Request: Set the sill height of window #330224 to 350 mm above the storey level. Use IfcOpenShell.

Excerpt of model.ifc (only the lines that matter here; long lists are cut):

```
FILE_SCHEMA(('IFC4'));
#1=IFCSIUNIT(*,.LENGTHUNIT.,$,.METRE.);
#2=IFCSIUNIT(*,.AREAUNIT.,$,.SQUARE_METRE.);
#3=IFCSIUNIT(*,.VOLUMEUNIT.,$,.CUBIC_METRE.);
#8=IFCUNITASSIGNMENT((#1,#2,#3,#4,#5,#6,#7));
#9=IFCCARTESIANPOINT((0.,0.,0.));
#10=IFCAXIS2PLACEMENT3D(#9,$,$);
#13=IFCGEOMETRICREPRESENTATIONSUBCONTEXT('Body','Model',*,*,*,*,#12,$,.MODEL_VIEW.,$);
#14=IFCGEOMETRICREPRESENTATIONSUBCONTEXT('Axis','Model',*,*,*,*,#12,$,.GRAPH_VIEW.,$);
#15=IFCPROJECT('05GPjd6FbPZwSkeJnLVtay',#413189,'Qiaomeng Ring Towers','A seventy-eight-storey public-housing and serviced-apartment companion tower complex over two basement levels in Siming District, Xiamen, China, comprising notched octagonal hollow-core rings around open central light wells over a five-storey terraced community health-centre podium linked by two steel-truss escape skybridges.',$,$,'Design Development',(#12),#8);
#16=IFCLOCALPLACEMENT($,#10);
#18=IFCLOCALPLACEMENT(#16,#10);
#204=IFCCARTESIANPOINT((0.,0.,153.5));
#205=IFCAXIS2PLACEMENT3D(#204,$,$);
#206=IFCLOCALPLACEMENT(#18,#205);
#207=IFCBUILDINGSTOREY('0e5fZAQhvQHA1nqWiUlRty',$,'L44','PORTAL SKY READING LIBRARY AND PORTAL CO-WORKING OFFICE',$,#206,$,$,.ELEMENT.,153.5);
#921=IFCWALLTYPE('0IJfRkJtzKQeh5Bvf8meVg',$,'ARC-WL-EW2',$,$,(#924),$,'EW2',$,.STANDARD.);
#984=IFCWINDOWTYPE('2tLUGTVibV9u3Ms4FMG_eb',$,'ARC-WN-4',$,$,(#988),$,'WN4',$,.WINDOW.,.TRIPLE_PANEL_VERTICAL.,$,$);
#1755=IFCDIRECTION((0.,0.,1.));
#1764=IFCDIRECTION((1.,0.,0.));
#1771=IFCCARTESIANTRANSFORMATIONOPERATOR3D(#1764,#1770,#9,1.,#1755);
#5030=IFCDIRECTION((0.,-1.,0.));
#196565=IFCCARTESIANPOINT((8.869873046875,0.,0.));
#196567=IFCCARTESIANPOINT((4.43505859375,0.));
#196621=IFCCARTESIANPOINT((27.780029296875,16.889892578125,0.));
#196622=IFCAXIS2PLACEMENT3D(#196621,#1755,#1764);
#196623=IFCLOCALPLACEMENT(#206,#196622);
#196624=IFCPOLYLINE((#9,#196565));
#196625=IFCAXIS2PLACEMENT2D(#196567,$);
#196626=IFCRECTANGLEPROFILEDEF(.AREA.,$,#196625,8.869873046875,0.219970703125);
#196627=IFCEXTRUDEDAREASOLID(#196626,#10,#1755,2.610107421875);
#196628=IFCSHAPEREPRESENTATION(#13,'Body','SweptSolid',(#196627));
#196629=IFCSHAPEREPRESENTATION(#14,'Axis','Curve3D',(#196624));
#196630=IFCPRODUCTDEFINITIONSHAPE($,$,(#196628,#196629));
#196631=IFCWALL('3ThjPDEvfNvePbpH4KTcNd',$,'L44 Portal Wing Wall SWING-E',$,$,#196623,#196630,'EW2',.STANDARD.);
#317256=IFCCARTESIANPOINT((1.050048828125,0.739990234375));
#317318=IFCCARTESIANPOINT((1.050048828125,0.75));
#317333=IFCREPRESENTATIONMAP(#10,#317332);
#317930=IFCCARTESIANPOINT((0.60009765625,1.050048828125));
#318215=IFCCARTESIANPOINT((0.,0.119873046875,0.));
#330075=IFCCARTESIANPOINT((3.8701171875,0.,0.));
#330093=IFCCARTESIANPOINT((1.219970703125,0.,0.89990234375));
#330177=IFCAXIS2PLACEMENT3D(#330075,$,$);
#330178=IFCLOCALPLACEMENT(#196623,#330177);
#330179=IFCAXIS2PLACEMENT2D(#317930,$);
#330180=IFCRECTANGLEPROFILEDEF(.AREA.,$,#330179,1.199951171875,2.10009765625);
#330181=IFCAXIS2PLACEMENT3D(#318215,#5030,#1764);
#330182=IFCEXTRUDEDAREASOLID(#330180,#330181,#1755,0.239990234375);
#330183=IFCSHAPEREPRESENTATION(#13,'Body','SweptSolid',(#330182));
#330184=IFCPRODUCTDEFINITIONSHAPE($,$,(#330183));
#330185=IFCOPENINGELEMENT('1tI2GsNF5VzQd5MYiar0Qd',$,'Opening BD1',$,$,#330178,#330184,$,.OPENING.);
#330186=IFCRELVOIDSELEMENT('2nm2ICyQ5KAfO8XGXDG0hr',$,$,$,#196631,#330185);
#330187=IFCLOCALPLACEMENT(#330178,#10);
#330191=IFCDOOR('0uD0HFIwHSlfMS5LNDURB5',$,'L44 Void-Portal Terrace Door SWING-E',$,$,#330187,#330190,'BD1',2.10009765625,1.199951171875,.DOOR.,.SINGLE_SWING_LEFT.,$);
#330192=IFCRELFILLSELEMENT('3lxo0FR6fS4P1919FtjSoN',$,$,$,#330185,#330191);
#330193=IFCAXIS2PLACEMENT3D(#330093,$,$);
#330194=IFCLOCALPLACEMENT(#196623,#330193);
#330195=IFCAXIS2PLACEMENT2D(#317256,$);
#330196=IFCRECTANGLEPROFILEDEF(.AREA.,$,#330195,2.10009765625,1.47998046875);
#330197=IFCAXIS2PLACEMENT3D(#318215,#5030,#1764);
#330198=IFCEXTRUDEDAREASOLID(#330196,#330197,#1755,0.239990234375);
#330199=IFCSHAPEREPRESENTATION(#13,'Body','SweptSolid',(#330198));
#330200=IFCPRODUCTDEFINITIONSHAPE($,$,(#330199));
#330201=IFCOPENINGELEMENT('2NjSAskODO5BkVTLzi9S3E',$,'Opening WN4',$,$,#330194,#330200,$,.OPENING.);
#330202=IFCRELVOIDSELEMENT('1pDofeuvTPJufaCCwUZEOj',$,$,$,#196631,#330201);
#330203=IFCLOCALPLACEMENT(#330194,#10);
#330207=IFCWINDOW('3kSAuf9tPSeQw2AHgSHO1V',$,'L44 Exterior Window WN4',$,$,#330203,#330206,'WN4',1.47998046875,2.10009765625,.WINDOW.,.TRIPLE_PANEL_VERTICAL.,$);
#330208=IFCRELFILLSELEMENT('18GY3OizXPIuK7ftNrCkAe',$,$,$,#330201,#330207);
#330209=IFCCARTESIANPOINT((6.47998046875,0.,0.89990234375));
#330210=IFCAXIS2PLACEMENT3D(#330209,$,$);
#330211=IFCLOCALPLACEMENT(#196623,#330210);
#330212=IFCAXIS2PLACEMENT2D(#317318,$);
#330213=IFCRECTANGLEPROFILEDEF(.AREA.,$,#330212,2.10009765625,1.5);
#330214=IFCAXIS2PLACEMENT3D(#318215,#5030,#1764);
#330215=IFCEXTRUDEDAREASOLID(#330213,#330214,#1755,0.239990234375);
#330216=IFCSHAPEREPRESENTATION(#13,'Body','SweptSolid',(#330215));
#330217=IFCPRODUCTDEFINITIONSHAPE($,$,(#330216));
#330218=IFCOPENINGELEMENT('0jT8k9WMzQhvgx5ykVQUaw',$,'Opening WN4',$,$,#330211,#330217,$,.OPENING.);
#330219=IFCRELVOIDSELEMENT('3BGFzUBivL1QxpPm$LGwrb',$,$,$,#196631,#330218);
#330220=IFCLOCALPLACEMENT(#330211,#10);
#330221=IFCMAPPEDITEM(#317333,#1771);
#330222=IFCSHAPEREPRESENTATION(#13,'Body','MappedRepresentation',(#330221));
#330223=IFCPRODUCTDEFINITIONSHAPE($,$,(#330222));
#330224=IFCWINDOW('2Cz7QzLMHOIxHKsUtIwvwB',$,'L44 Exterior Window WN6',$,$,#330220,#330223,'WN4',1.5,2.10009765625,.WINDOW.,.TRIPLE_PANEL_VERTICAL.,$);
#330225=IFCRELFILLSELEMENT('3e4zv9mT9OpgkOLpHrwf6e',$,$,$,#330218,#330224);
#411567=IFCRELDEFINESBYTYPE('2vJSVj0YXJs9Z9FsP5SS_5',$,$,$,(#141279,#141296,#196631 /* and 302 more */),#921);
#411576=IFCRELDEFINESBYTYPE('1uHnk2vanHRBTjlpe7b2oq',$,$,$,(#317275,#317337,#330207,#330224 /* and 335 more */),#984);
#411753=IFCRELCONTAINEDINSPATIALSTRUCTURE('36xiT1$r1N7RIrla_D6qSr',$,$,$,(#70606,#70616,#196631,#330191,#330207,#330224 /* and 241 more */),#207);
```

```python
import numpy as np
import ifcopenshell
import ifcopenshell.api.geometry
import ifcopenshell.geom
import ifcopenshell.util.element
import ifcopenshell.util.placement
import ifcopenshell.util.shape
import ifcopenshell.util.unit

model = ifcopenshell.open("model.ifc")
unit_scale = ifcopenshell.util.unit.calculate_unit_scale(model)

window = model.by_guid("2Cz7QzLMHOIxHKsUtIwvwB")
opening = window.FillsVoids[0].RelatingOpeningElement
storey = ifcopenshell.util.element.get_container(window, ifc_class="IfcBuildingStorey")
level = ifcopenshell.util.placement.get_local_placement(storey.ObjectPlacement)[2, 3]

# The opening's origin need not be at the sill, so measure its lowest point.
shape = ifcopenshell.geom.create_shape(ifcopenshell.geom.settings(), opening)
bottom = ifcopenshell.util.shape.get_shape_bottom_elevation(shape, shape.geometry) / unit_scale
dz = level + 0.35 - bottom

shift = np.array([0.0, 0.0, dz])
# The window is placed relative to its opening, so it follows when the opening moves.
matrix = ifcopenshell.util.placement.get_local_placement(opening.ObjectPlacement)
matrix[:3, 3] += shift
ifcopenshell.api.geometry.edit_object_placement(
    model, product=opening, matrix=matrix, is_si=False, should_transform_children=True
)

print(f"moved by {dz * unit_scale:+.3f} m")

model.write("model_v2.ifc")
```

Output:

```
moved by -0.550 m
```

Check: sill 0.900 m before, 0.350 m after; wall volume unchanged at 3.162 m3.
